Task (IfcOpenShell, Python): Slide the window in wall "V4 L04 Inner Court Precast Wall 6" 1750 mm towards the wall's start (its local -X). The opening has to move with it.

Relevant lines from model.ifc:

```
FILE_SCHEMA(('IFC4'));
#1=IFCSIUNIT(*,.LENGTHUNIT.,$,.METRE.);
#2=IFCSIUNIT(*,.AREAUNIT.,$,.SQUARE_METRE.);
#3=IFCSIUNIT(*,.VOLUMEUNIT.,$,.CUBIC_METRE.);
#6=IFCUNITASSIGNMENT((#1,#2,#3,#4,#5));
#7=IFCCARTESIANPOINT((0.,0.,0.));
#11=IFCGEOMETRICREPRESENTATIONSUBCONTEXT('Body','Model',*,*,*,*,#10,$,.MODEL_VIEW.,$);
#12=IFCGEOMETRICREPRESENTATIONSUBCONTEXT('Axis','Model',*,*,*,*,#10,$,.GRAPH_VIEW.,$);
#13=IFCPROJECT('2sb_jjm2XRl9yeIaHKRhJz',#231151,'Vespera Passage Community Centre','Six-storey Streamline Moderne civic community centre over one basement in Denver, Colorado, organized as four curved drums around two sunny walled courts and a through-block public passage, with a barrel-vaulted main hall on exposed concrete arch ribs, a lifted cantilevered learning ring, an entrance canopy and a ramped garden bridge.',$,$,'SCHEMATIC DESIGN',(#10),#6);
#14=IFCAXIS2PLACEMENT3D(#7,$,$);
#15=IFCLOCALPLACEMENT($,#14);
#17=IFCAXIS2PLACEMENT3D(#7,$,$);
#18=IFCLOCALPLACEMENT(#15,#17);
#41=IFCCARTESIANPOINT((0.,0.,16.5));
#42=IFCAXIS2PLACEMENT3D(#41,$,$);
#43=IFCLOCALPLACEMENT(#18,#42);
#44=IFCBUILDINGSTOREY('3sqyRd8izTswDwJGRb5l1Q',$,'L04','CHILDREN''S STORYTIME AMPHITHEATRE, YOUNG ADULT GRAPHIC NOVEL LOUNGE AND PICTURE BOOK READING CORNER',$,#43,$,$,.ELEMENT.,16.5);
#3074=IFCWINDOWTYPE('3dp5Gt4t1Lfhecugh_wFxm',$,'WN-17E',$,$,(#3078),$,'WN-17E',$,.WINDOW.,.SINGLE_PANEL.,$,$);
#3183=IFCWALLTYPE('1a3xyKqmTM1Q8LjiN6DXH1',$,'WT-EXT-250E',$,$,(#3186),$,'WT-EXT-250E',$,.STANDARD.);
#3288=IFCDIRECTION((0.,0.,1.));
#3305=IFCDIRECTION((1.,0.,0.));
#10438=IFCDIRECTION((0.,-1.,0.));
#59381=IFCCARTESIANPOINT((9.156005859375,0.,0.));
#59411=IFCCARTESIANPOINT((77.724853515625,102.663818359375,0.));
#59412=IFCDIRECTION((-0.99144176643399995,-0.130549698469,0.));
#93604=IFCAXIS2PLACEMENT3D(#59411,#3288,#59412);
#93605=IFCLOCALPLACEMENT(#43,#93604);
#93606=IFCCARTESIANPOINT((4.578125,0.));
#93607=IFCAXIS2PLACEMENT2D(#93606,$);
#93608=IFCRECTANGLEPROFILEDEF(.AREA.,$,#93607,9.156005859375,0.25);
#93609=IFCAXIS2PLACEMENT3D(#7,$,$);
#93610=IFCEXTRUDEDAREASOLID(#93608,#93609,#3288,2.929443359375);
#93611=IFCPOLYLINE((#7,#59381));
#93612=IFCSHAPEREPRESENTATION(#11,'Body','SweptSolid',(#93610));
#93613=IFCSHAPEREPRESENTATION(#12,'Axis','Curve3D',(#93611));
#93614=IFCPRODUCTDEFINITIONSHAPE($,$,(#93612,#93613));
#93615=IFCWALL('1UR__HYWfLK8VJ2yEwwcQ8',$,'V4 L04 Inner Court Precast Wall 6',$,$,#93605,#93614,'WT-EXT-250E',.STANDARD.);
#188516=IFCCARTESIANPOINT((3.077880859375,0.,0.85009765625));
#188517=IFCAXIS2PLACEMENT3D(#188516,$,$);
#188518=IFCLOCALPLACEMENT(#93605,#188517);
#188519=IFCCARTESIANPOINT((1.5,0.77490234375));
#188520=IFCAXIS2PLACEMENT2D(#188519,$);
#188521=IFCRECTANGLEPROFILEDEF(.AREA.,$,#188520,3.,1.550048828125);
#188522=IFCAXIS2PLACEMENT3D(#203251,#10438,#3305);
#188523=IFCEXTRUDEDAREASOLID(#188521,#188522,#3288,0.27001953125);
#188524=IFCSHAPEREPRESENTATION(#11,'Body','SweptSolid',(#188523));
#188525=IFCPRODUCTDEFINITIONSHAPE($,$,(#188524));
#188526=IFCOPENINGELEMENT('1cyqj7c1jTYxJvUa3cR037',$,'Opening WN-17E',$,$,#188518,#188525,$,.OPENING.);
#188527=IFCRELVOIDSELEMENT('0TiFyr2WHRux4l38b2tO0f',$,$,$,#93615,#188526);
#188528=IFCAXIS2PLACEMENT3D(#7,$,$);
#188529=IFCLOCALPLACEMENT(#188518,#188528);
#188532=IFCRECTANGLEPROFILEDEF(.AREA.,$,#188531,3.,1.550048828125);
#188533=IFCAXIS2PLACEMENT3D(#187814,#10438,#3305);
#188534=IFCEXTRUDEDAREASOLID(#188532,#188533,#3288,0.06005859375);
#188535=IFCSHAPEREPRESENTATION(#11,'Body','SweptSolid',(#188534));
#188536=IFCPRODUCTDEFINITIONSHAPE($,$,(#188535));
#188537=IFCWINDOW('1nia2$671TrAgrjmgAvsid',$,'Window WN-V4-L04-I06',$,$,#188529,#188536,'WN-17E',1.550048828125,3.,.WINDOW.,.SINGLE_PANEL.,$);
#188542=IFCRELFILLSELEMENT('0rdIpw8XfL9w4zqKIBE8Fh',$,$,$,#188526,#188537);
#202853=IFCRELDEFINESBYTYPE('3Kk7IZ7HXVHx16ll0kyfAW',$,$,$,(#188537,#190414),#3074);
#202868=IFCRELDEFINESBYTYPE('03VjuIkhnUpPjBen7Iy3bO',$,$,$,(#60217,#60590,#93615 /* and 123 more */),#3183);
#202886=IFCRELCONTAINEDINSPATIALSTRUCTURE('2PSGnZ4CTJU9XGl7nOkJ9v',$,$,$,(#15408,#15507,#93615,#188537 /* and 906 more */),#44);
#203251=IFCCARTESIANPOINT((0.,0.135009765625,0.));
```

```python
import ifcopenshell
import ifcopenshell.api.geometry
import ifcopenshell.util.placement
import ifcopenshell.util.unit

model = ifcopenshell.open("model.ifc")
unit_scale = ifcopenshell.util.unit.calculate_unit_scale(model)

window = model.by_guid("1nia2$671TrAgrjmgAvsid")
opening = window.FillsVoids[0].RelatingOpeningElement
wall = opening.VoidsElements[0].RelatingBuildingElement

wall_matrix = ifcopenshell.util.placement.get_local_placement(wall.ObjectPlacement)
shift = wall_matrix[:3, 0] * -1.75 / unit_scale
before = ifcopenshell.util.placement.get_local_placement(window.ObjectPlacement)[:3, 3].copy()

# The window is placed relative to its opening, so it follows when the opening moves.
matrix = ifcopenshell.util.placement.get_local_placement(opening.ObjectPlacement)
matrix[:3, 3] += shift
ifcopenshell.api.geometry.edit_object_placement(
    model, product=opening, matrix=matrix, is_si=False, should_transform_children=True
)

after = ifcopenshell.util.placement.get_local_placement(window.ObjectPlacement)[:3, 3]
print("window moved by", (after - before).round(3) + 0.0)

model.write("model_updated.ifc")
```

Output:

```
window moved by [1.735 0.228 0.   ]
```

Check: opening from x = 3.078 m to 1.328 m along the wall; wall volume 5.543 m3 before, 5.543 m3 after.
